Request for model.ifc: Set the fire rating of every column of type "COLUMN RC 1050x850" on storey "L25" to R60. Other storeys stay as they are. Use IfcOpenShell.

First a look at what the model holds.

```python
import ifcopenshell
import ifcopenshell.util.element

model = ifcopenshell.open("model.ifc")
print(model.schema)
storey = next(s for s in model.by_type("IfcBuildingStorey") if s.Name == "L25")
columns = [e for e in ifcopenshell.util.element.get_decomposition(storey) if e.is_a("IfcColumn")]
seen = {}
for e in columns:
    element_type = ifcopenshell.util.element.get_type(e)
    key = (element_type.Name if element_type != e and element_type else None, ifcopenshell.util.element.get_pset(e, "Pset_ColumnCommon", "FireRating"))
    seen[key] = seen.get(key, 0) + 1
for (name, value), count in sorted(seen.items(), key=str):
    print(count, "x", name, "|", value)
```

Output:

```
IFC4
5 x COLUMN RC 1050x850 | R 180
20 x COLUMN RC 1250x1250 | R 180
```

```python
import ifcopenshell
import ifcopenshell.api.pset
import ifcopenshell.util.element

model = ifcopenshell.open("model.ifc")

storey = next(s for s in model.by_type("IfcBuildingStorey") if s.Name == "L25")
columns = [e for e in ifcopenshell.util.element.get_decomposition(storey) if e.is_a("IfcColumn")]

count = 0
for e in columns:
    element_type = ifcopenshell.util.element.get_type(e)
    if element_type in (None, e) or element_type.Name != "COLUMN RC 1050x850":
        continue
    found = ifcopenshell.util.element.get_pset(e, "Pset_ColumnCommon", should_inherit=False)
    if found:
        pset = model.by_id(found["id"])
        if len(ifcopenshell.util.element.get_elements_by_pset(pset)) > 1:
            pset = ifcopenshell.api.pset.unshare_pset(model, products=[e], pset=pset)[0]
    else:
        pset = ifcopenshell.api.pset.add_pset(model, product=e, name="Pset_ColumnCommon")
    ifcopenshell.api.pset.edit_pset(model, pset=pset, properties={"FireRating": "R60"})
    count += 1

print(count, "columns updated")

model.write("model_edited.ifc")
```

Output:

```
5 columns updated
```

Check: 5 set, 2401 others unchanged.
